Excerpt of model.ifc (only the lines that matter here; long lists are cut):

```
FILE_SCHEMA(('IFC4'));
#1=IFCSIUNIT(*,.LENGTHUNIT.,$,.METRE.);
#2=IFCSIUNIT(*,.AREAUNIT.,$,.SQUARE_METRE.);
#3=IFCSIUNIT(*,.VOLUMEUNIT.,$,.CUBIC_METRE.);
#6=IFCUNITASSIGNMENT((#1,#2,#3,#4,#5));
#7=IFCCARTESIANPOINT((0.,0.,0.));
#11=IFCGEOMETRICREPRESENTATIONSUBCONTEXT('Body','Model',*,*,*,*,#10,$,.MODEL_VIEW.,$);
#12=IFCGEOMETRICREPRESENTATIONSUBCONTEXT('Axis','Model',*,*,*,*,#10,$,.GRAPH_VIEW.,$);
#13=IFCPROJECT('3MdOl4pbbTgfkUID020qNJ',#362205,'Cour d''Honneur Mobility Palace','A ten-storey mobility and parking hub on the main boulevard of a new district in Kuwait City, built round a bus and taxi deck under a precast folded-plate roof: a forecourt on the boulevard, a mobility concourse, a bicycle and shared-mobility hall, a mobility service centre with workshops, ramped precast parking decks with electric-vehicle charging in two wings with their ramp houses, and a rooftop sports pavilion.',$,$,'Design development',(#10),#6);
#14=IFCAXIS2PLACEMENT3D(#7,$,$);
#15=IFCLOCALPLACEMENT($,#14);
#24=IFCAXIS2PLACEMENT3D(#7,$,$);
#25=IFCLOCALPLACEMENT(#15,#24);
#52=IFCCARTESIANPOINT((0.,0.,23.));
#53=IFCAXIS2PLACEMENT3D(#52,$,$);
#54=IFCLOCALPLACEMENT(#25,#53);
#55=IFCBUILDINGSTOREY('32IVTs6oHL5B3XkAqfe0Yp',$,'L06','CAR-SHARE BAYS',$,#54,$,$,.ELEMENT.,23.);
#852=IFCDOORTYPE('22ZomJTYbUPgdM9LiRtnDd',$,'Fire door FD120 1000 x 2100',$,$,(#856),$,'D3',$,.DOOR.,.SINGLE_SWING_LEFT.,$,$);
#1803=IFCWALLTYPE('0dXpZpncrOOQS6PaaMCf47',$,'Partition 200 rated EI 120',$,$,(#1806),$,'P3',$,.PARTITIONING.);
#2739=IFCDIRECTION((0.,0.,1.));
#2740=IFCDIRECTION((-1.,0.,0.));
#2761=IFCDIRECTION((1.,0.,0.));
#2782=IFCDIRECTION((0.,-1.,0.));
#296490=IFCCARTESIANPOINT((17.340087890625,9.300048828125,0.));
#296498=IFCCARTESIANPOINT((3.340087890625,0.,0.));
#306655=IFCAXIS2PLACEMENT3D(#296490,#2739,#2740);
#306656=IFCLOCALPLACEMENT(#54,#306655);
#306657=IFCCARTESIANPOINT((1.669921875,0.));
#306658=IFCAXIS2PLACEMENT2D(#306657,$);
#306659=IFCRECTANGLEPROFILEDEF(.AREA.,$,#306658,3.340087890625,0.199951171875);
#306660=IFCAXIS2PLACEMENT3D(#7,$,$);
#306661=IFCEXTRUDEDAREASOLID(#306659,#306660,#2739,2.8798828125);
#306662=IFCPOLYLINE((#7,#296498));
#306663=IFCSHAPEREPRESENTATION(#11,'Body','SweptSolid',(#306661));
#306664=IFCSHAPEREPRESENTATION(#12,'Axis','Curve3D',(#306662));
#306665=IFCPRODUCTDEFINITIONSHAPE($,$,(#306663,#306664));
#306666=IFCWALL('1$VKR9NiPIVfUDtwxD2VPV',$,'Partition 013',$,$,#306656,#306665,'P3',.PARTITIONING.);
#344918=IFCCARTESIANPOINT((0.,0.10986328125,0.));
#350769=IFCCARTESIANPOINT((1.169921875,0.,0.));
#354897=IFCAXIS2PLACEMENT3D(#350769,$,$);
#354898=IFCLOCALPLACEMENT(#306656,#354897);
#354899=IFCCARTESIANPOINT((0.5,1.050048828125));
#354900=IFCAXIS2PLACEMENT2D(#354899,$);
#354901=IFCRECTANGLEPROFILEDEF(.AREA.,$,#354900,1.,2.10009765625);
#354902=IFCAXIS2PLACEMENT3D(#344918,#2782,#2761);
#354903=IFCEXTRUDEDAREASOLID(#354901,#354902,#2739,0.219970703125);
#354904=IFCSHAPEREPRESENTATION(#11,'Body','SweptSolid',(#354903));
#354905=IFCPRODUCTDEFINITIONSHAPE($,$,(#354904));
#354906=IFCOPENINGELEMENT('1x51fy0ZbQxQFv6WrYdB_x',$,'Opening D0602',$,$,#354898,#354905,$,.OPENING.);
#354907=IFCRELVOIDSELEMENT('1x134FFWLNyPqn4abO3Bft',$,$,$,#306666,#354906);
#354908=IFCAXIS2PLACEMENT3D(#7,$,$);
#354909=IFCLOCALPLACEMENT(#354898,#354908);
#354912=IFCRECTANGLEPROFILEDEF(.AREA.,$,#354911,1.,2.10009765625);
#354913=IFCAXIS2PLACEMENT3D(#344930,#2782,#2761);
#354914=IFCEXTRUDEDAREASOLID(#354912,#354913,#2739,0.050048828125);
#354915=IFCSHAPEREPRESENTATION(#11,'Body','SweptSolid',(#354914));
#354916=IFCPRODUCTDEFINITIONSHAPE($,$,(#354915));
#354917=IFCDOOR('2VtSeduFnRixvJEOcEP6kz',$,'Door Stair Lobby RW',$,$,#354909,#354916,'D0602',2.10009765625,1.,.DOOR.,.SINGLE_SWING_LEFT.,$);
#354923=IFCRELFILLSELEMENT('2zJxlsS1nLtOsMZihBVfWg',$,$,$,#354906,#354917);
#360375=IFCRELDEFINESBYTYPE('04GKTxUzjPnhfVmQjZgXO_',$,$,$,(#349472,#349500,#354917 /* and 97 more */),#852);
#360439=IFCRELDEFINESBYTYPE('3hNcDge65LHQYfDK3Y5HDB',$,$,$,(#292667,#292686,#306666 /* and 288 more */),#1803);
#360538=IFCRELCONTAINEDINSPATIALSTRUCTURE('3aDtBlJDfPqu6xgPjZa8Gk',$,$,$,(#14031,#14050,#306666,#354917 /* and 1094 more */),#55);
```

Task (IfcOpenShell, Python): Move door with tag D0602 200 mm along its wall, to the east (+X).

```python
import ifcopenshell
import ifcopenshell.api.geometry
import ifcopenshell.util.placement

model = ifcopenshell.open("model.ifc")

door = model.by_guid("2VtSeduFnRixvJEOcEP6kz")
opening = door.FillsVoids[0].RelatingOpeningElement
wall = opening.VoidsElements[0].RelatingBuildingElement

wall_matrix = ifcopenshell.util.placement.get_local_placement(wall.ObjectPlacement)
shift = wall_matrix[:3, 0] * -0.2
before = ifcopenshell.util.placement.get_local_placement(door.ObjectPlacement)[:3, 3].copy()

# The door is placed relative to its opening, so it follows when the opening moves.
matrix = ifcopenshell.util.placement.get_local_placement(opening.ObjectPlacement)
matrix[:3, 3] += shift
ifcopenshell.api.geometry.edit_object_placement(
    model, product=opening, matrix=matrix, is_si=False, should_transform_children=True
)

after = ifcopenshell.util.placement.get_local_placement(door.ObjectPlacement)[:3, 3]
print("door moved by", (after - before).round(3) + 0.0)

model.write("model_rev.ifc")
```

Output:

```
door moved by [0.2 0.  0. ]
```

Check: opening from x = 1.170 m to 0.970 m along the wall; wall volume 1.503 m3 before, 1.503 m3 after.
